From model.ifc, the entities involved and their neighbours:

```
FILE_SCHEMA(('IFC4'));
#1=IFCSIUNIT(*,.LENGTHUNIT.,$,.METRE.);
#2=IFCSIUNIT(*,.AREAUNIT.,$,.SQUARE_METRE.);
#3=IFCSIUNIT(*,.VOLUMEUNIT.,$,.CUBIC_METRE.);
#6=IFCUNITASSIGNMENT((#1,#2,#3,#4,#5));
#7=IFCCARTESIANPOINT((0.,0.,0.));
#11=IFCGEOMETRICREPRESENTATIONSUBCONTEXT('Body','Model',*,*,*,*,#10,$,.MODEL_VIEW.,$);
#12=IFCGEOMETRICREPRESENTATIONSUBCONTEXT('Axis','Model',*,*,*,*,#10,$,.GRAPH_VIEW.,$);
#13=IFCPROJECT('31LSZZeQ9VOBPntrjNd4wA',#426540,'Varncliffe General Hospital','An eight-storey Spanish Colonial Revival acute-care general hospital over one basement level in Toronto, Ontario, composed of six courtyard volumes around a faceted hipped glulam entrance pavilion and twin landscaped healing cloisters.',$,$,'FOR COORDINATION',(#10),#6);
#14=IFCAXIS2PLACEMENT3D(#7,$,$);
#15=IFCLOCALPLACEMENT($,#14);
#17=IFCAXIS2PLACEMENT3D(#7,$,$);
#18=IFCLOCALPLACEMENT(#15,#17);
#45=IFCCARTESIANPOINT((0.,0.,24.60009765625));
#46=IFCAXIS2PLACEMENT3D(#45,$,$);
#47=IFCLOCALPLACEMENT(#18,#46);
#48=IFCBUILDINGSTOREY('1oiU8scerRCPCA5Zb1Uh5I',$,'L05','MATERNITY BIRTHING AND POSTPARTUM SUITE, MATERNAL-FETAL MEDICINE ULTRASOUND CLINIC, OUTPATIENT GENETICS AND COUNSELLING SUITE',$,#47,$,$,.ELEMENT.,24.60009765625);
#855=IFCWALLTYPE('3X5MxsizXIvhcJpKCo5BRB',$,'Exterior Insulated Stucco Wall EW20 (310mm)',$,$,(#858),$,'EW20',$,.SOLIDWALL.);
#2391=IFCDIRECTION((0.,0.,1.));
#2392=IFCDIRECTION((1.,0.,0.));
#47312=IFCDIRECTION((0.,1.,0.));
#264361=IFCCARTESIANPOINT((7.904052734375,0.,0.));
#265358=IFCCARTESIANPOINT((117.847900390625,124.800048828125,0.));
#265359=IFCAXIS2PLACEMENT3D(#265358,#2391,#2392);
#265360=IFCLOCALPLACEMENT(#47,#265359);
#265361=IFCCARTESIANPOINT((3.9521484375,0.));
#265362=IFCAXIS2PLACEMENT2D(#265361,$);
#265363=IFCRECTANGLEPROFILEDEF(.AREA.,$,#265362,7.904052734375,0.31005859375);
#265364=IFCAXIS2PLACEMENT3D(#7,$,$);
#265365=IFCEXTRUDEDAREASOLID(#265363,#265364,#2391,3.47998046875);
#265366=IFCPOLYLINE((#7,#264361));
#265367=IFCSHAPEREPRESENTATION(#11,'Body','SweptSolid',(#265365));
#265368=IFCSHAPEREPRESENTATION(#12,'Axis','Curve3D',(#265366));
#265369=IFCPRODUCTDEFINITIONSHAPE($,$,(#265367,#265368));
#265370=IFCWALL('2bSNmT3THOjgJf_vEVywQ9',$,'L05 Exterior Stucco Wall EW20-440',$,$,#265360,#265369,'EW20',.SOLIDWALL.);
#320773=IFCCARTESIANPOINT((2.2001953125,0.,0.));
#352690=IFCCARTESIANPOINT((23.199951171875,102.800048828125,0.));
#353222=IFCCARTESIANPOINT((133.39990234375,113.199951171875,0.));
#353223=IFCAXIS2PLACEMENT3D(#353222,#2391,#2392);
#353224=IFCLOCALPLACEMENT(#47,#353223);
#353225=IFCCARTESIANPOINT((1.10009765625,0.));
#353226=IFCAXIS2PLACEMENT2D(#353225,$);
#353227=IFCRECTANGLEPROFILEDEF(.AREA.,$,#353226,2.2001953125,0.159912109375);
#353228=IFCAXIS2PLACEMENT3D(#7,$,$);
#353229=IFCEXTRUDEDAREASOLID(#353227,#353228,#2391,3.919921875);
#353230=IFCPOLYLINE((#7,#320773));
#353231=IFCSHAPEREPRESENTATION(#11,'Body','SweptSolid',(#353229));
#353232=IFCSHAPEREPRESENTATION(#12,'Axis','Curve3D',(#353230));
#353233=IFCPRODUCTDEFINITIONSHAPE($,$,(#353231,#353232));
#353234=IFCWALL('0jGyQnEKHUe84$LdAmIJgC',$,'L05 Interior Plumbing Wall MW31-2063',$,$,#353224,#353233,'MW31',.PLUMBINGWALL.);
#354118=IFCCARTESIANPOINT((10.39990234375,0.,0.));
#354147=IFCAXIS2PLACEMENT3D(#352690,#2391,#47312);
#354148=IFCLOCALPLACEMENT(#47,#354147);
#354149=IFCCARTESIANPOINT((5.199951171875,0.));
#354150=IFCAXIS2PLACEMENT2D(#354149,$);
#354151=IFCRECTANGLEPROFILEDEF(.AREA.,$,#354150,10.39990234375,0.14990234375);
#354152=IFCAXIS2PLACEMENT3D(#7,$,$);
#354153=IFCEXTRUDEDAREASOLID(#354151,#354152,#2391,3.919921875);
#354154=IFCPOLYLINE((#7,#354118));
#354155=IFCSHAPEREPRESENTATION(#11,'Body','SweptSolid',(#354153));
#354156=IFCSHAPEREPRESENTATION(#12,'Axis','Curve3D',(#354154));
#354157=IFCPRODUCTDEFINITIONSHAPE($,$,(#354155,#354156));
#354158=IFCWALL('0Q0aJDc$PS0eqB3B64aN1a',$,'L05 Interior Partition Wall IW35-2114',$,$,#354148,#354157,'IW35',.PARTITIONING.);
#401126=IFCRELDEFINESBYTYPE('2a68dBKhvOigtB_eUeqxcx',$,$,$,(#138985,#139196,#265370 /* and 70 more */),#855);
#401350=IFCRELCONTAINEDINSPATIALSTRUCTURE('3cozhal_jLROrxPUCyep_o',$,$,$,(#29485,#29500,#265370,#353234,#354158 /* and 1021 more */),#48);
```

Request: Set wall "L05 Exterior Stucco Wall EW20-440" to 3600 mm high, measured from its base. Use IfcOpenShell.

```python
import ifcopenshell
import ifcopenshell.geom
import ifcopenshell.util.representation
import ifcopenshell.util.shape
import ifcopenshell.util.unit

model = ifcopenshell.open("model.ifc")
unit_scale = ifcopenshell.util.unit.calculate_unit_scale(model)
settings = ifcopenshell.geom.settings()


def volume(element):
    """Net volume in cubic metres, openings subtracted."""
    shape = ifcopenshell.geom.create_shape(settings, element)
    return ifcopenshell.util.shape.get_volume(shape.geometry)


wall = model.by_id(265370)
before = volume(wall)

body = ifcopenshell.util.representation.get_representation(wall, "Model", "Body")
solid = body.Items[0]
old_height = solid.Depth
solid.Depth = 3.6 / unit_scale
after = volume(wall)

print(f"height {old_height:g} -> {solid.Depth:g}, volume {before:.3f} -> {after:.3f} m3")

model.write("model_updated.ifc")
```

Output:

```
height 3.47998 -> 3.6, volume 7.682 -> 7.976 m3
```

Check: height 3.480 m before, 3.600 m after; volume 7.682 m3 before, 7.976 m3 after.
